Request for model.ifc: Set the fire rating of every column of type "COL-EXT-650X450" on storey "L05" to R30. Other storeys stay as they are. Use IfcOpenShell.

First a look at what the model holds.

```python
import ifcopenshell
import ifcopenshell.util.element

model = ifcopenshell.open("model.ifc")
print(model.schema)
storey = next(s for s in model.by_type("IfcBuildingStorey") if s.Name == "L05")
columns = [e for e in ifcopenshell.util.element.get_decomposition(storey) if e.is_a("IfcColumn")]
seen = {}
for e in columns:
    element_type = ifcopenshell.util.element.get_type(e)
    key = (element_type.Name if element_type != e and element_type else None, ifcopenshell.util.element.get_pset(e, "Pset_ColumnCommon", "FireRating"))
    seen[key] = seen.get(key, 0) + 1
for (name, value), count in sorted(seen.items(), key=str):
    print(count, "x", name, "|", value)
```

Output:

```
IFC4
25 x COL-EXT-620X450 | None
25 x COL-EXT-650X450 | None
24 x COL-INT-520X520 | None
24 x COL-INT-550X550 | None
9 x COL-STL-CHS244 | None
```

```python
import ifcopenshell
import ifcopenshell.api.pset
import ifcopenshell.util.element

model = ifcopenshell.open("model.ifc")

storey = next(s for s in model.by_type("IfcBuildingStorey") if s.Name == "L05")
columns = [e for e in ifcopenshell.util.element.get_decomposition(storey) if e.is_a("IfcColumn")]

count = 0
for e in columns:
    element_type = ifcopenshell.util.element.get_type(e)
    if element_type in (None, e) or element_type.Name != "COL-EXT-650X450":
        continue
    # add_pset returns the element's existing set when there is one.
    pset = ifcopenshell.api.pset.add_pset(model, product=e, name="Pset_ColumnCommon")
    ifcopenshell.api.pset.edit_pset(model, pset=pset, properties={"FireRating": "R30"})
    count += 1

print(count, "columns updated")

model.write("model-out.ifc")
```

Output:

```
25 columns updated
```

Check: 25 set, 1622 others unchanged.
